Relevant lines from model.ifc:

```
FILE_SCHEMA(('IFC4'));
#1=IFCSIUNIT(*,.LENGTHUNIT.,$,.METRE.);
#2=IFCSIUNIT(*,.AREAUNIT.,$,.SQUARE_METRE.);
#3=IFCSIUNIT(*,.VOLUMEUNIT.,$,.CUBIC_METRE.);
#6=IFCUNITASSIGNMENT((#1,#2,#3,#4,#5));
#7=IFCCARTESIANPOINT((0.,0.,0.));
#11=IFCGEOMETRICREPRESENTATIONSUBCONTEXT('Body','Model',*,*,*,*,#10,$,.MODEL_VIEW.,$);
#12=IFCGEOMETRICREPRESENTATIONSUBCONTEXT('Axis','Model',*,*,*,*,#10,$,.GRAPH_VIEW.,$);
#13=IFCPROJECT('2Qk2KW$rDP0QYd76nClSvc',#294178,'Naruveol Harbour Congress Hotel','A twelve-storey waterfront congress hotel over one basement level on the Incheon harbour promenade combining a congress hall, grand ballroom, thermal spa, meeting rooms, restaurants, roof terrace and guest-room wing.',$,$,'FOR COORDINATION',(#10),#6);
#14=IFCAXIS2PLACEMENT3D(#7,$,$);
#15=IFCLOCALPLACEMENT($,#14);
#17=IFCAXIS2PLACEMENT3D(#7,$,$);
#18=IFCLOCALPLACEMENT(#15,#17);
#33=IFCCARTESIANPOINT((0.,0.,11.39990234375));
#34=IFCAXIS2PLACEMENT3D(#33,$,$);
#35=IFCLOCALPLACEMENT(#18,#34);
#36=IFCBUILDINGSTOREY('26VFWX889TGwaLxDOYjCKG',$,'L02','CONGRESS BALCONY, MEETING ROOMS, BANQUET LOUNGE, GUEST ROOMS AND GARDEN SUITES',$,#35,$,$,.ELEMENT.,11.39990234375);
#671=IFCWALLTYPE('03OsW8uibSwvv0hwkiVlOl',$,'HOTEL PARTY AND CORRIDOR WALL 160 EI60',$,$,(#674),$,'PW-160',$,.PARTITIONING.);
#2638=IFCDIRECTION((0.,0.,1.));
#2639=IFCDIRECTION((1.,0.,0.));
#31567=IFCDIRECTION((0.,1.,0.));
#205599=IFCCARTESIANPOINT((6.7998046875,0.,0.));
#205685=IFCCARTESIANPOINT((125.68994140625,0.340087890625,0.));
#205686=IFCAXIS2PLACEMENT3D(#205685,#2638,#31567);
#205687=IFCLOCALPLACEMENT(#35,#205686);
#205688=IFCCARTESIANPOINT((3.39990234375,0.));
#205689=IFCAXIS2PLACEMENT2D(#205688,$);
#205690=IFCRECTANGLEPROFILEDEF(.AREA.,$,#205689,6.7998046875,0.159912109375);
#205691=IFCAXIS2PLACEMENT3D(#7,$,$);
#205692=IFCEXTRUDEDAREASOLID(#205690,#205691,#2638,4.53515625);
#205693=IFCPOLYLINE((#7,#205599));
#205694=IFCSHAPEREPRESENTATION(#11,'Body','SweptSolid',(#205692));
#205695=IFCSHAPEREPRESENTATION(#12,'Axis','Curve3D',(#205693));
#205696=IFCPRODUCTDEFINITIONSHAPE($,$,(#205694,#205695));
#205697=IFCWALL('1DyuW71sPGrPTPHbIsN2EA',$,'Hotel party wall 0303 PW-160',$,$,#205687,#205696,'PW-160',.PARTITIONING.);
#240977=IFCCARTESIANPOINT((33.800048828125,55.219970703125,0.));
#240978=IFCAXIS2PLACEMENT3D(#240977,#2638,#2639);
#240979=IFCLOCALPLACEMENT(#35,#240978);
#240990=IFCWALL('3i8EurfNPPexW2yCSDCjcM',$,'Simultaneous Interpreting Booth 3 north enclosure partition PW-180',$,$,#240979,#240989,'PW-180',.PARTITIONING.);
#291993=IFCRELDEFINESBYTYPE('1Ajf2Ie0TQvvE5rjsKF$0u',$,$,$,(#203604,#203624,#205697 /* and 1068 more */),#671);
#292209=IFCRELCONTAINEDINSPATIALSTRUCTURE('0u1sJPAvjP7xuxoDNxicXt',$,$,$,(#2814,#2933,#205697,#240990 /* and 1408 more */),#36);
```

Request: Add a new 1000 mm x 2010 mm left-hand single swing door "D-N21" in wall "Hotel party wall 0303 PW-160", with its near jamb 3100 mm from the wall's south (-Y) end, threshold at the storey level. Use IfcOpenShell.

```python
import numpy as np
import ifcopenshell
import ifcopenshell.api.feature
import ifcopenshell.api.geometry
import ifcopenshell.api.root
import ifcopenshell.api.spatial
import ifcopenshell.geom
import ifcopenshell.util.element
import ifcopenshell.util.placement
import ifcopenshell.util.representation
import ifcopenshell.util.shape
import ifcopenshell.util.unit

model = ifcopenshell.open("model.ifc")
unit_scale = ifcopenshell.util.unit.calculate_unit_scale(model)
settings = ifcopenshell.geom.settings()


def volume(element):
    """Net volume in cubic metres, openings subtracted."""
    shape = ifcopenshell.geom.create_shape(settings, element)
    return ifcopenshell.util.shape.get_volume(shape.geometry)


wall = model.by_guid("1DyuW71sPGrPTPHbIsN2EA")
storey = ifcopenshell.util.element.get_container(wall, ifc_class="IfcBuildingStorey")
context = ifcopenshell.util.representation.get_context(model, "Model", "Body", "MODEL_VIEW")
before = volume(wall)

width, height, from_end, sill = 1, 2.01, 3.1, 0.0  # metres

# The wall runs along its own X axis, and the end named is its -X end.
wall_shape = ifcopenshell.geom.create_shape(settings, wall)
x, y, z = ifcopenshell.util.shape.get_vertices(wall_shape.geometry).T
start = x.min() + from_end
face, thickness = float(y.min()), float(y.max() - y.min())
wall_matrix = ifcopenshell.util.placement.get_local_placement(wall.ObjectPlacement)
level = ifcopenshell.util.placement.get_local_placement(storey.ObjectPlacement)[2, 3]


def in_wall(x, y):
    """Placement at x, y metres in the wall's axes, at sill height."""
    matrix = wall_matrix.copy()
    matrix[:, 3] = wall_matrix @ np.array([x / unit_scale, y / unit_scale, 0.0, 1.0])
    matrix[2, 3] = level + sill / unit_scale
    return matrix


# Opening: a box that overshoots both wall faces by 50 mm.
opening = ifcopenshell.api.root.create_entity(model, ifc_class="IfcOpeningElement", predefined_type="OPENING")
box = ifcopenshell.api.geometry.add_wall_representation(
    model, context=context, length=width, height=height, thickness=thickness + 0.1
)
ifcopenshell.api.geometry.assign_representation(model, product=opening, representation=box)
ifcopenshell.api.geometry.edit_object_placement(model, product=opening, matrix=in_wall(start, face - 0.05), is_si=False)
ifcopenshell.api.feature.add_feature(model, feature=opening, element=wall)

door = ifcopenshell.api.root.create_entity(model, ifc_class="IfcDoor", name="D-N21", predefined_type="DOOR")
door.OverallWidth, door.OverallHeight = width / unit_scale, height / unit_scale
door.OperationType = "SINGLE_SWING_LEFT"
body = ifcopenshell.api.geometry.add_door_representation(
    model,
    context=context,
    overall_width=door.OverallWidth,
    overall_height=door.OverallHeight,
    operation_type="SINGLE_SWING_LEFT",
    lining_properties={"LiningDepth": thickness / unit_scale, "ThresholdDepth": thickness / unit_scale},
)
ifcopenshell.api.geometry.assign_representation(model, product=door, representation=body)
ifcopenshell.api.spatial.assign_container(model, products=[door], relating_structure=storey)
ifcopenshell.api.feature.add_filling(model, opening=opening, element=door)

# The lining spans the wall, so the door starts at the wall face.
ifcopenshell.api.geometry.edit_object_placement(model, product=door, matrix=in_wall(start, face), is_si=False)

after = volume(wall)

print(f"wall volume {before:.3f} -> {after:.3f} m3")

model.write("model_updated.ifc")
```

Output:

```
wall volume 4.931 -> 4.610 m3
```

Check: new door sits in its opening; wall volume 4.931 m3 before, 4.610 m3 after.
